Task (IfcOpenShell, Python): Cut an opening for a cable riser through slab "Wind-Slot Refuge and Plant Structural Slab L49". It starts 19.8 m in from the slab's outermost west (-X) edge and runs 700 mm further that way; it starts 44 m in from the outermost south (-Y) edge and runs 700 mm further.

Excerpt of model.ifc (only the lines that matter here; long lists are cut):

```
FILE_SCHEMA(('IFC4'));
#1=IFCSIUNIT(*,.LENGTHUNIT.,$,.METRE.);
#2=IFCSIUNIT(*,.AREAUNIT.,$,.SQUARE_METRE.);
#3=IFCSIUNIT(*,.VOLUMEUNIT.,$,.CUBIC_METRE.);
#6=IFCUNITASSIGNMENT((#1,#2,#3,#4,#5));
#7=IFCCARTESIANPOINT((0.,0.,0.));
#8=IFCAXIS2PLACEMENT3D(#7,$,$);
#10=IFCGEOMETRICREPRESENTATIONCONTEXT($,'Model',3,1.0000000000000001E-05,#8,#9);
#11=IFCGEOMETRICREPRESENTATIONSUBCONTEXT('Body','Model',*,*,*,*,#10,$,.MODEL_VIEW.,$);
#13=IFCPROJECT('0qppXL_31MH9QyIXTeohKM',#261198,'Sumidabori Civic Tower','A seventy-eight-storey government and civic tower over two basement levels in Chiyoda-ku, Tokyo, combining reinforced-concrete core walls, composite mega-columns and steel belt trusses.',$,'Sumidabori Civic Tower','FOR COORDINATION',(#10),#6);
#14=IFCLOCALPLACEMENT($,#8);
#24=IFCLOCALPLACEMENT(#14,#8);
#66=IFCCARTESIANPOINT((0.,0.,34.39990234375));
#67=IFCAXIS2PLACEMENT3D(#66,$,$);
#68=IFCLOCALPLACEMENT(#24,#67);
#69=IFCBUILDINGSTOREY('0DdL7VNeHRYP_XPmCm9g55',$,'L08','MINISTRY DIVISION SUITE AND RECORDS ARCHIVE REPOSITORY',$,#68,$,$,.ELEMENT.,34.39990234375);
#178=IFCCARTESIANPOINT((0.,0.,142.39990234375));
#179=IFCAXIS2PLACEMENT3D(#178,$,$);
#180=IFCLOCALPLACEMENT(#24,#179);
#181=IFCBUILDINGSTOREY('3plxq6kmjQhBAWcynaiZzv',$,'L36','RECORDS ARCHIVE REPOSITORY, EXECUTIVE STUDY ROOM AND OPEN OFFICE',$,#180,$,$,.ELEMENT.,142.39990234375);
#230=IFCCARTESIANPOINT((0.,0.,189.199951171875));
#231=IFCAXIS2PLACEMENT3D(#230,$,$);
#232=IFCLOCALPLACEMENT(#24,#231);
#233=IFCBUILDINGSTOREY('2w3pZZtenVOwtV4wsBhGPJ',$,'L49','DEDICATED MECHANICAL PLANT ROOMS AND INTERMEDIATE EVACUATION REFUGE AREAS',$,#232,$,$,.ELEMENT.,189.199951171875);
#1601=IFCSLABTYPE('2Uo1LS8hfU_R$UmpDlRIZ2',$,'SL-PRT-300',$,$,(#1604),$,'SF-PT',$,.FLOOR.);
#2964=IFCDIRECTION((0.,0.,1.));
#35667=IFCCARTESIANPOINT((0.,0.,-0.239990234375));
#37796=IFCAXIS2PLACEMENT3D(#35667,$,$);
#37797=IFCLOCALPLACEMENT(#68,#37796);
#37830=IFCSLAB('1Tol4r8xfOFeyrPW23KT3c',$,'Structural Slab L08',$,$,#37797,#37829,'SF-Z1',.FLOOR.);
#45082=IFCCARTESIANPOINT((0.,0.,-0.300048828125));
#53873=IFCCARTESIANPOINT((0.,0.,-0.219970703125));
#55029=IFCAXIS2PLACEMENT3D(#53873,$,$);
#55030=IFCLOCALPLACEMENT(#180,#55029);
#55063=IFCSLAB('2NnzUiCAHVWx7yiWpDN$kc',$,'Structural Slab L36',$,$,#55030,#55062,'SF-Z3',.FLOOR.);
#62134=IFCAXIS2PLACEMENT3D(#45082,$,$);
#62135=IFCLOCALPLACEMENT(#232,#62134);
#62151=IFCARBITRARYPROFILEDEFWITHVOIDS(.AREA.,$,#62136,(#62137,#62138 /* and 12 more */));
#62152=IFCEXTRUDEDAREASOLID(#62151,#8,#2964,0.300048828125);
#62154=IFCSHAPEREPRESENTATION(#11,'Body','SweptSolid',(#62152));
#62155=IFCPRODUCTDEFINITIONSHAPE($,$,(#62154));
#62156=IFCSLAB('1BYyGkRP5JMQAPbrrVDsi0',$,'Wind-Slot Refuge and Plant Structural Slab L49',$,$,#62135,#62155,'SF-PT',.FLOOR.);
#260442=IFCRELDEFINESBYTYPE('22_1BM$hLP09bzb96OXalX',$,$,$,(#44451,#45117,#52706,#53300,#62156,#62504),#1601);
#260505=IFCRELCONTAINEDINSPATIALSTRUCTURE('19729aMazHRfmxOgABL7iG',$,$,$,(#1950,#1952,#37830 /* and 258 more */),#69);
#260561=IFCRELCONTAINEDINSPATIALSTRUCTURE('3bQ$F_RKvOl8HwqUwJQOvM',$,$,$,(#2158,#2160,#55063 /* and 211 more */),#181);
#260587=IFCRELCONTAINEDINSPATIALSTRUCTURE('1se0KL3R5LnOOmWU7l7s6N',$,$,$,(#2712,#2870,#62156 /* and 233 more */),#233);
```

```python
import numpy as np
import ifcopenshell
import ifcopenshell.api.feature
import ifcopenshell.api.geometry
import ifcopenshell.api.root
import ifcopenshell.geom
import ifcopenshell.util.placement
import ifcopenshell.util.representation
import ifcopenshell.util.shape
import ifcopenshell.util.unit

model = ifcopenshell.open("model.ifc")
unit_scale = ifcopenshell.util.unit.calculate_unit_scale(model)
settings = ifcopenshell.geom.settings()


def volume(element):
    """Net volume in cubic metres, openings subtracted."""
    shape = ifcopenshell.geom.create_shape(settings, element)
    return ifcopenshell.util.shape.get_volume(shape.geometry)


slab = model.by_guid("1BYyGkRP5JMQAPbrrVDsi0")
before = volume(slab)

# Extent in the slab's own axes, in metres. The edges named are its -X and -Y sides.
slab_shape = ifcopenshell.geom.create_shape(settings, slab)
vertices = ifcopenshell.util.shape.get_vertices(slab_shape.geometry)
x_min, y_min, bottom = vertices.min(axis=0)
top = vertices[:, 2].max()

opening = ifcopenshell.api.root.create_entity(model, ifc_class="IfcOpeningElement", name="Cable riser opening", predefined_type="OPENING")
context = ifcopenshell.util.representation.get_context(model, "Model", "Body", "MODEL_VIEW")
width, depth = 0.7, 0.7
outline = [(0.0, 0.0), (width, 0.0), (width, depth), (0.0, depth), (0.0, 0.0)]
# Overshoot both faces by 50 mm so the cut is clean.
shape = ifcopenshell.api.geometry.add_slab_representation(
    model, context=context, depth=top - bottom + 0.1, polyline=outline
)
ifcopenshell.api.geometry.assign_representation(model, product=opening, representation=shape)

matrix = ifcopenshell.util.placement.get_local_placement(slab.ObjectPlacement)
matrix[:, 3] = matrix @ np.append(np.array([x_min + 19.8, y_min + 44, bottom - 0.05]) / unit_scale, 1.0)
ifcopenshell.api.geometry.edit_object_placement(model, product=opening, matrix=matrix, is_si=False)
ifcopenshell.api.feature.add_feature(model, feature=opening, element=slab)

after = volume(slab)

print(f"slab volume {before:.3f} -> {after:.3f} m3")

model.write("model_edited.ifc")
```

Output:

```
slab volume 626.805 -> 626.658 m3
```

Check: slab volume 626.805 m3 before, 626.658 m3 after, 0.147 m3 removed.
